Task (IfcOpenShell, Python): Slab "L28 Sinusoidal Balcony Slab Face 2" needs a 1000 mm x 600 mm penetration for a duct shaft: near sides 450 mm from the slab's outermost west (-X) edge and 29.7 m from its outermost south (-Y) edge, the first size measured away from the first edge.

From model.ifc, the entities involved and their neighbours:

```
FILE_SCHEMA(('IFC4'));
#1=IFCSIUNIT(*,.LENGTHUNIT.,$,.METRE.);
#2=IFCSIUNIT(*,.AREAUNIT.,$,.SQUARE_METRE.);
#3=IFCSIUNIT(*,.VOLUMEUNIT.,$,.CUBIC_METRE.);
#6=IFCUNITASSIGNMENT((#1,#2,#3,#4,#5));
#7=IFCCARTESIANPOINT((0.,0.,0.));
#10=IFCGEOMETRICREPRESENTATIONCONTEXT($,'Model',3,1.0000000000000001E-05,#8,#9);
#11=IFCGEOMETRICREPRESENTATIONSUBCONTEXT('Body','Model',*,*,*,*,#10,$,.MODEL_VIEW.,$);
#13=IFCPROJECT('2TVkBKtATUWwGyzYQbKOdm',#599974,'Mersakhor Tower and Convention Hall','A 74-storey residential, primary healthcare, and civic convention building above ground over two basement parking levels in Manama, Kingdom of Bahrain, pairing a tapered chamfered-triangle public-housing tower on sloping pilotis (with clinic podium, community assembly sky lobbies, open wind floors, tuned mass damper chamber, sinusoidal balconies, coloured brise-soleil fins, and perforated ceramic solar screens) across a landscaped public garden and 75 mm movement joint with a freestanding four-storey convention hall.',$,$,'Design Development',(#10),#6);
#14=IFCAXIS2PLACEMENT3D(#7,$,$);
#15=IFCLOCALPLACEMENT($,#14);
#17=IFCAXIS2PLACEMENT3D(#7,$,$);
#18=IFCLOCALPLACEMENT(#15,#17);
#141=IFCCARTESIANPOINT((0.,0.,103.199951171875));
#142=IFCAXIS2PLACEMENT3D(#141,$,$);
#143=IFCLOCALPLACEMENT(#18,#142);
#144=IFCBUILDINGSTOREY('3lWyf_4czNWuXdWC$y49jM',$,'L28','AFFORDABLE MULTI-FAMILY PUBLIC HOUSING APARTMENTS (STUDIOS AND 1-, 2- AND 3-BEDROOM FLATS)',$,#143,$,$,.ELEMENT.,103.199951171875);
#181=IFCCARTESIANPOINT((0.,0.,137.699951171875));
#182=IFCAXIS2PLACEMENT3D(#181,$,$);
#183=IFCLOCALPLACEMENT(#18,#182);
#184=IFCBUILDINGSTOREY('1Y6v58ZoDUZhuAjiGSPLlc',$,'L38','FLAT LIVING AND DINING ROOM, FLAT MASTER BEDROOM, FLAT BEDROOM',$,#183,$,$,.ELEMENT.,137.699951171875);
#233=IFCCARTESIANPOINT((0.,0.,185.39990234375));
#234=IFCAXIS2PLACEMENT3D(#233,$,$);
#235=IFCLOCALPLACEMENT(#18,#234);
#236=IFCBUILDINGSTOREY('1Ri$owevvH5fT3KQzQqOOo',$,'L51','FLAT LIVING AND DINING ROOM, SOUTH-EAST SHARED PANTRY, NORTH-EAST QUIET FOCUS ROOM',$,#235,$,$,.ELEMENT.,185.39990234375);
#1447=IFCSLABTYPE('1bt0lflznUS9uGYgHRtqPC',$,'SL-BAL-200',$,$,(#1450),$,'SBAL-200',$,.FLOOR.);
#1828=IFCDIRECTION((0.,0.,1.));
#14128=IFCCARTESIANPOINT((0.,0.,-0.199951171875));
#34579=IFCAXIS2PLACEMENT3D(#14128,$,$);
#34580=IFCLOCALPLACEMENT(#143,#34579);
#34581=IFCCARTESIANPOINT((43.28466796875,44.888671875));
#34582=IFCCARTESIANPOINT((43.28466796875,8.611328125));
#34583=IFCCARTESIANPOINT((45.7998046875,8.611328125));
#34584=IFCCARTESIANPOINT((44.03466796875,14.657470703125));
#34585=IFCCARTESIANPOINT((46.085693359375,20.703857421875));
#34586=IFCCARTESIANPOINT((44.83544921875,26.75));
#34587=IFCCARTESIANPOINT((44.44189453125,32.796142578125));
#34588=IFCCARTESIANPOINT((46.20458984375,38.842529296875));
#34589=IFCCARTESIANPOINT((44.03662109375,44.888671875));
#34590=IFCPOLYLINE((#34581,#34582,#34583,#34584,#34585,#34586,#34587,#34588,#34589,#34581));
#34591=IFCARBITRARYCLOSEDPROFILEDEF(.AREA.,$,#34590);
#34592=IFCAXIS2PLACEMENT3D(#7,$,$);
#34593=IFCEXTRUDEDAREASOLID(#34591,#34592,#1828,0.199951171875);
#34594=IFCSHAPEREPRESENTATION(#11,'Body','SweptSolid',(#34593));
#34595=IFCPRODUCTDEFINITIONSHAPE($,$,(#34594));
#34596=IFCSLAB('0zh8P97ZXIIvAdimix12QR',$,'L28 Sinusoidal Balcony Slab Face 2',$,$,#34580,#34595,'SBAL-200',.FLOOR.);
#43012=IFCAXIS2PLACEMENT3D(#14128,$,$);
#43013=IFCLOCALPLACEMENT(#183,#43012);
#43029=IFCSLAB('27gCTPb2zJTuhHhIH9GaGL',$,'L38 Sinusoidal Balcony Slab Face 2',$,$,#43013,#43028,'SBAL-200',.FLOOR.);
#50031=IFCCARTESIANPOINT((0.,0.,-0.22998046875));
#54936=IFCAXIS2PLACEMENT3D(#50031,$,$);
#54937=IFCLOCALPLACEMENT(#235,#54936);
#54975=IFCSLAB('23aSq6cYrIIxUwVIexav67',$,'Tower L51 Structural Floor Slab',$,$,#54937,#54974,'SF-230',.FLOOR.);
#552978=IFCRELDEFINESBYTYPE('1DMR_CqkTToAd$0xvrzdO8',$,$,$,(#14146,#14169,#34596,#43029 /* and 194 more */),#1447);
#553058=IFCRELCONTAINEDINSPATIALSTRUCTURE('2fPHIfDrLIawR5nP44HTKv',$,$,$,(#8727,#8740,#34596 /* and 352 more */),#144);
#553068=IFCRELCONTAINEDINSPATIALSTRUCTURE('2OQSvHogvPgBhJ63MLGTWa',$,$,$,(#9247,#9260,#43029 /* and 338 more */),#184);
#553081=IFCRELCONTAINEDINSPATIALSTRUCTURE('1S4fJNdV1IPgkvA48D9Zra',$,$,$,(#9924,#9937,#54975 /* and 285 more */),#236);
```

```python
import numpy as np
import ifcopenshell
import ifcopenshell.api.feature
import ifcopenshell.api.geometry
import ifcopenshell.api.root
import ifcopenshell.geom
import ifcopenshell.util.placement
import ifcopenshell.util.representation
import ifcopenshell.util.shape
import ifcopenshell.util.unit

model = ifcopenshell.open("model.ifc")
unit_scale = ifcopenshell.util.unit.calculate_unit_scale(model)
settings = ifcopenshell.geom.settings()


def volume(element):
    """Net volume in cubic metres, openings subtracted."""
    shape = ifcopenshell.geom.create_shape(settings, element)
    return ifcopenshell.util.shape.get_volume(shape.geometry)


slab = model.by_id(34596)
before = volume(slab)

# Extent in the slab's own axes, in metres. The edges named are its -X and -Y sides.
slab_shape = ifcopenshell.geom.create_shape(settings, slab)
vertices = ifcopenshell.util.shape.get_vertices(slab_shape.geometry)
x_min, y_min, bottom = vertices.min(axis=0)
top = vertices[:, 2].max()

opening = ifcopenshell.api.root.create_entity(model, ifc_class="IfcOpeningElement", name="Duct shaft opening", predefined_type="OPENING")
context = ifcopenshell.util.representation.get_context(model, "Model", "Body", "MODEL_VIEW")
width, depth = 1, 0.6
outline = [(0.0, 0.0), (width, 0.0), (width, depth), (0.0, depth), (0.0, 0.0)]
# Overshoot both faces by 50 mm so the cut is clean.
shape = ifcopenshell.api.geometry.add_slab_representation(
    model, context=context, depth=top - bottom + 0.1, polyline=outline
)
ifcopenshell.api.geometry.assign_representation(model, product=opening, representation=shape)

matrix = ifcopenshell.util.placement.get_local_placement(slab.ObjectPlacement)
matrix[:, 3] = matrix @ np.append(np.array([x_min + 0.45, y_min + 29.7, bottom - 0.05]) / unit_scale, 1.0)
ifcopenshell.api.geometry.edit_object_placement(model, product=opening, matrix=matrix, is_si=False)
ifcopenshell.api.feature.add_feature(model, feature=opening, element=slab)

after = volume(slab)

print(f"slab volume {before:.3f} -> {after:.3f} m3")

model.write("model_edited.ifc")
```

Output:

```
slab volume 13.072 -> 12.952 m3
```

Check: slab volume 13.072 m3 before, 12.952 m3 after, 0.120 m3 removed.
